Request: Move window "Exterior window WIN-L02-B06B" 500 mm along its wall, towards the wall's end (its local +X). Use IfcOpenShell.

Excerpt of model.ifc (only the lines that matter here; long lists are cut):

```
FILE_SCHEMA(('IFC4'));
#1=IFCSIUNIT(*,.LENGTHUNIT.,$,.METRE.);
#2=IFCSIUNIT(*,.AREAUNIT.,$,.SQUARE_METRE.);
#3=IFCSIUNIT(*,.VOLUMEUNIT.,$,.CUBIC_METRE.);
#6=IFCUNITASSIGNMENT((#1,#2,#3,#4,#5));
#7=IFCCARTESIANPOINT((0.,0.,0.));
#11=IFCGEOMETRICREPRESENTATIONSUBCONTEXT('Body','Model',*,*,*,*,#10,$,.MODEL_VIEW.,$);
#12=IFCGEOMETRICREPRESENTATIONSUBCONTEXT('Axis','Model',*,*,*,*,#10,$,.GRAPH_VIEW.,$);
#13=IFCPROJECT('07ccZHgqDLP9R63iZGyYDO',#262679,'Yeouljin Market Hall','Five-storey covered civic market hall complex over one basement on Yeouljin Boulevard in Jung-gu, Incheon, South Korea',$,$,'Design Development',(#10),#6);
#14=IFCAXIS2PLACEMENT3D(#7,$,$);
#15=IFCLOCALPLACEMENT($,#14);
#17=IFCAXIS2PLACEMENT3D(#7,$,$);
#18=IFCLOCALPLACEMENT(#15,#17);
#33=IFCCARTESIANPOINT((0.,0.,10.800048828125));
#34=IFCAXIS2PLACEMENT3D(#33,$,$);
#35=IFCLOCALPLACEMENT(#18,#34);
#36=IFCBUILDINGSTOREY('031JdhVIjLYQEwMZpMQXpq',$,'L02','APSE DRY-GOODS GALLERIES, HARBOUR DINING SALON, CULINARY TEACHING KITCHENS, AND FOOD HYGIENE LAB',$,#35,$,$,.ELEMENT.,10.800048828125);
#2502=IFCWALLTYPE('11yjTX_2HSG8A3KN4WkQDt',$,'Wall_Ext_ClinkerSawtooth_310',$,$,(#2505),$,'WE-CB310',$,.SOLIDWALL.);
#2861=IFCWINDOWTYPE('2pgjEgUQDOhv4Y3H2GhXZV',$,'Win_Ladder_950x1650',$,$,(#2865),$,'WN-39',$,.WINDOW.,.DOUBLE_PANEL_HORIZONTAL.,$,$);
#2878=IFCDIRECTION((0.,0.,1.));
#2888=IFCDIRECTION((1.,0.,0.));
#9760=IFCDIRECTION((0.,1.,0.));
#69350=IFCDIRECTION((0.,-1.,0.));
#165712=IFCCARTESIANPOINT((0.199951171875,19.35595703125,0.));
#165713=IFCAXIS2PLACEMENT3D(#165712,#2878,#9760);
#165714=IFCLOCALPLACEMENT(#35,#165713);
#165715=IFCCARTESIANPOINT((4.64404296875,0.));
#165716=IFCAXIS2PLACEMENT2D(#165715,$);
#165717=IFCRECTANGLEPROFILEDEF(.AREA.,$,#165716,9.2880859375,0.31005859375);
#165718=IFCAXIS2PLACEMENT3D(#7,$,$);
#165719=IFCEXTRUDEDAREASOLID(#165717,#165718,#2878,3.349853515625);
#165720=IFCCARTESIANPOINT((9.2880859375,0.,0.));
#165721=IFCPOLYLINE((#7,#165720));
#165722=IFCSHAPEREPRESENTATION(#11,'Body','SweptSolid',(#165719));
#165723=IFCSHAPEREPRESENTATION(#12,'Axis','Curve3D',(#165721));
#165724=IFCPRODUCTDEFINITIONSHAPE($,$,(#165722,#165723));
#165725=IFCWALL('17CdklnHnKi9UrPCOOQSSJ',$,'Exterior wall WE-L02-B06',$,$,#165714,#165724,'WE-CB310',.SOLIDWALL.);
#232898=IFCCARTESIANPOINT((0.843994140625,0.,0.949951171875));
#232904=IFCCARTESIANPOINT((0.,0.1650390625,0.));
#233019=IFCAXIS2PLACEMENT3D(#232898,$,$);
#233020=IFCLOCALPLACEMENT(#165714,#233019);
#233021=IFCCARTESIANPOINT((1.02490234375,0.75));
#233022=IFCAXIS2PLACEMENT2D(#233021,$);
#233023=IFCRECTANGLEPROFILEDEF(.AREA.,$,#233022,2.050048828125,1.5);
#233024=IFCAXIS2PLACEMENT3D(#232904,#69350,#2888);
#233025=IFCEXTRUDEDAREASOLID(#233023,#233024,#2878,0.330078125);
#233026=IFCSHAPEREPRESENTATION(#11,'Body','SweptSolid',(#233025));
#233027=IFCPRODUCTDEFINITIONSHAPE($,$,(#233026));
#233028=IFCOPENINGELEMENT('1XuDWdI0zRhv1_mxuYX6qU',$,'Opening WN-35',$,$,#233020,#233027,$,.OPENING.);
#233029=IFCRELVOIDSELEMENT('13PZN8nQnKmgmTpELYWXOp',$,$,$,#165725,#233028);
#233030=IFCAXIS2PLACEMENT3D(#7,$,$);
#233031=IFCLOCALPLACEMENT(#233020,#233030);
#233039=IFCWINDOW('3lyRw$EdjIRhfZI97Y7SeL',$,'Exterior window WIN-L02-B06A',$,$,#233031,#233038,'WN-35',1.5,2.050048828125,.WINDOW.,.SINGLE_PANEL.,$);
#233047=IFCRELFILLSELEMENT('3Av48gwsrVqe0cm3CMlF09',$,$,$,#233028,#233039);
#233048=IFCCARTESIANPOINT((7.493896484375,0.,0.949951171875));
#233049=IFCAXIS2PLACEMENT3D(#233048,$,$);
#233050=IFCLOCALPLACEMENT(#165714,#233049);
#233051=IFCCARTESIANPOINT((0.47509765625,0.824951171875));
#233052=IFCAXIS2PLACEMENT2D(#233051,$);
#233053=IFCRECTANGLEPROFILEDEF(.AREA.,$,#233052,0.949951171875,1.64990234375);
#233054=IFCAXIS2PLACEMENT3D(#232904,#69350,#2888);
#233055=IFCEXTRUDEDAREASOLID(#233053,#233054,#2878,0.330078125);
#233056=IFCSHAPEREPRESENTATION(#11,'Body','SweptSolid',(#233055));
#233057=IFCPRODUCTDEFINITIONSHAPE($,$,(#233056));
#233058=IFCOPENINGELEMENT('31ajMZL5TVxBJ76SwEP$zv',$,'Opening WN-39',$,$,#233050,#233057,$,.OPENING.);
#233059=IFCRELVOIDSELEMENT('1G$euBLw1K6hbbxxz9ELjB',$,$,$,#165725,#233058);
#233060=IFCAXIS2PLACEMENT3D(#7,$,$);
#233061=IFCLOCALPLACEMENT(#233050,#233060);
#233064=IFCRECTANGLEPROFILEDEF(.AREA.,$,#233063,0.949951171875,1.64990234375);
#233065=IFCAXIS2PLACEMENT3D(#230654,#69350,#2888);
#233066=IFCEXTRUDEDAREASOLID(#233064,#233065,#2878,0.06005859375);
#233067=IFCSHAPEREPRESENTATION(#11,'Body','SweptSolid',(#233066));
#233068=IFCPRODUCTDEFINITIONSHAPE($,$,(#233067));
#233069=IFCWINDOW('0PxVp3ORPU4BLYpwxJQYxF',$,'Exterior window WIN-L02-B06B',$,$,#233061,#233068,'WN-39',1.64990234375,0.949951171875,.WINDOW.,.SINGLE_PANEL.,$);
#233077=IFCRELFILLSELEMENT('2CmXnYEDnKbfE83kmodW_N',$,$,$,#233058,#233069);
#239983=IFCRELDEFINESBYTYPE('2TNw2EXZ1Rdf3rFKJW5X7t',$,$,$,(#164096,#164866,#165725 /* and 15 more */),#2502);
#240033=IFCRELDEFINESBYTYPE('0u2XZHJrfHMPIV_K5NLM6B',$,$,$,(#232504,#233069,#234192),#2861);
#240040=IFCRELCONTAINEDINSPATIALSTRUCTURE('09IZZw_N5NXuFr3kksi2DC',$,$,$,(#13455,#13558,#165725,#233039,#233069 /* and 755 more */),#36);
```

```python
import ifcopenshell
import ifcopenshell.api.geometry
import ifcopenshell.util.placement

model = ifcopenshell.open("model.ifc")

window = model.by_guid("0PxVp3ORPU4BLYpwxJQYxF")
opening = window.FillsVoids[0].RelatingOpeningElement
wall = opening.VoidsElements[0].RelatingBuildingElement

wall_matrix = ifcopenshell.util.placement.get_local_placement(wall.ObjectPlacement)
shift = wall_matrix[:3, 0] * 0.5
before = ifcopenshell.util.placement.get_local_placement(window.ObjectPlacement)[:3, 3].copy()

# The window is placed relative to its opening, so it follows when the opening moves.
matrix = ifcopenshell.util.placement.get_local_placement(opening.ObjectPlacement)
matrix[:3, 3] += shift
ifcopenshell.api.geometry.edit_object_placement(
    model, product=opening, matrix=matrix, is_si=False, should_transform_children=True
)

after = ifcopenshell.util.placement.get_local_placement(window.ObjectPlacement)[:3, 3]
print("window moved by", (after - before).round(3) + 0.0)

model.write("model_edited.ifc")
```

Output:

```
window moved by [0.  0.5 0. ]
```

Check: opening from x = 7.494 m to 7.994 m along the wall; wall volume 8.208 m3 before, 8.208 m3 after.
